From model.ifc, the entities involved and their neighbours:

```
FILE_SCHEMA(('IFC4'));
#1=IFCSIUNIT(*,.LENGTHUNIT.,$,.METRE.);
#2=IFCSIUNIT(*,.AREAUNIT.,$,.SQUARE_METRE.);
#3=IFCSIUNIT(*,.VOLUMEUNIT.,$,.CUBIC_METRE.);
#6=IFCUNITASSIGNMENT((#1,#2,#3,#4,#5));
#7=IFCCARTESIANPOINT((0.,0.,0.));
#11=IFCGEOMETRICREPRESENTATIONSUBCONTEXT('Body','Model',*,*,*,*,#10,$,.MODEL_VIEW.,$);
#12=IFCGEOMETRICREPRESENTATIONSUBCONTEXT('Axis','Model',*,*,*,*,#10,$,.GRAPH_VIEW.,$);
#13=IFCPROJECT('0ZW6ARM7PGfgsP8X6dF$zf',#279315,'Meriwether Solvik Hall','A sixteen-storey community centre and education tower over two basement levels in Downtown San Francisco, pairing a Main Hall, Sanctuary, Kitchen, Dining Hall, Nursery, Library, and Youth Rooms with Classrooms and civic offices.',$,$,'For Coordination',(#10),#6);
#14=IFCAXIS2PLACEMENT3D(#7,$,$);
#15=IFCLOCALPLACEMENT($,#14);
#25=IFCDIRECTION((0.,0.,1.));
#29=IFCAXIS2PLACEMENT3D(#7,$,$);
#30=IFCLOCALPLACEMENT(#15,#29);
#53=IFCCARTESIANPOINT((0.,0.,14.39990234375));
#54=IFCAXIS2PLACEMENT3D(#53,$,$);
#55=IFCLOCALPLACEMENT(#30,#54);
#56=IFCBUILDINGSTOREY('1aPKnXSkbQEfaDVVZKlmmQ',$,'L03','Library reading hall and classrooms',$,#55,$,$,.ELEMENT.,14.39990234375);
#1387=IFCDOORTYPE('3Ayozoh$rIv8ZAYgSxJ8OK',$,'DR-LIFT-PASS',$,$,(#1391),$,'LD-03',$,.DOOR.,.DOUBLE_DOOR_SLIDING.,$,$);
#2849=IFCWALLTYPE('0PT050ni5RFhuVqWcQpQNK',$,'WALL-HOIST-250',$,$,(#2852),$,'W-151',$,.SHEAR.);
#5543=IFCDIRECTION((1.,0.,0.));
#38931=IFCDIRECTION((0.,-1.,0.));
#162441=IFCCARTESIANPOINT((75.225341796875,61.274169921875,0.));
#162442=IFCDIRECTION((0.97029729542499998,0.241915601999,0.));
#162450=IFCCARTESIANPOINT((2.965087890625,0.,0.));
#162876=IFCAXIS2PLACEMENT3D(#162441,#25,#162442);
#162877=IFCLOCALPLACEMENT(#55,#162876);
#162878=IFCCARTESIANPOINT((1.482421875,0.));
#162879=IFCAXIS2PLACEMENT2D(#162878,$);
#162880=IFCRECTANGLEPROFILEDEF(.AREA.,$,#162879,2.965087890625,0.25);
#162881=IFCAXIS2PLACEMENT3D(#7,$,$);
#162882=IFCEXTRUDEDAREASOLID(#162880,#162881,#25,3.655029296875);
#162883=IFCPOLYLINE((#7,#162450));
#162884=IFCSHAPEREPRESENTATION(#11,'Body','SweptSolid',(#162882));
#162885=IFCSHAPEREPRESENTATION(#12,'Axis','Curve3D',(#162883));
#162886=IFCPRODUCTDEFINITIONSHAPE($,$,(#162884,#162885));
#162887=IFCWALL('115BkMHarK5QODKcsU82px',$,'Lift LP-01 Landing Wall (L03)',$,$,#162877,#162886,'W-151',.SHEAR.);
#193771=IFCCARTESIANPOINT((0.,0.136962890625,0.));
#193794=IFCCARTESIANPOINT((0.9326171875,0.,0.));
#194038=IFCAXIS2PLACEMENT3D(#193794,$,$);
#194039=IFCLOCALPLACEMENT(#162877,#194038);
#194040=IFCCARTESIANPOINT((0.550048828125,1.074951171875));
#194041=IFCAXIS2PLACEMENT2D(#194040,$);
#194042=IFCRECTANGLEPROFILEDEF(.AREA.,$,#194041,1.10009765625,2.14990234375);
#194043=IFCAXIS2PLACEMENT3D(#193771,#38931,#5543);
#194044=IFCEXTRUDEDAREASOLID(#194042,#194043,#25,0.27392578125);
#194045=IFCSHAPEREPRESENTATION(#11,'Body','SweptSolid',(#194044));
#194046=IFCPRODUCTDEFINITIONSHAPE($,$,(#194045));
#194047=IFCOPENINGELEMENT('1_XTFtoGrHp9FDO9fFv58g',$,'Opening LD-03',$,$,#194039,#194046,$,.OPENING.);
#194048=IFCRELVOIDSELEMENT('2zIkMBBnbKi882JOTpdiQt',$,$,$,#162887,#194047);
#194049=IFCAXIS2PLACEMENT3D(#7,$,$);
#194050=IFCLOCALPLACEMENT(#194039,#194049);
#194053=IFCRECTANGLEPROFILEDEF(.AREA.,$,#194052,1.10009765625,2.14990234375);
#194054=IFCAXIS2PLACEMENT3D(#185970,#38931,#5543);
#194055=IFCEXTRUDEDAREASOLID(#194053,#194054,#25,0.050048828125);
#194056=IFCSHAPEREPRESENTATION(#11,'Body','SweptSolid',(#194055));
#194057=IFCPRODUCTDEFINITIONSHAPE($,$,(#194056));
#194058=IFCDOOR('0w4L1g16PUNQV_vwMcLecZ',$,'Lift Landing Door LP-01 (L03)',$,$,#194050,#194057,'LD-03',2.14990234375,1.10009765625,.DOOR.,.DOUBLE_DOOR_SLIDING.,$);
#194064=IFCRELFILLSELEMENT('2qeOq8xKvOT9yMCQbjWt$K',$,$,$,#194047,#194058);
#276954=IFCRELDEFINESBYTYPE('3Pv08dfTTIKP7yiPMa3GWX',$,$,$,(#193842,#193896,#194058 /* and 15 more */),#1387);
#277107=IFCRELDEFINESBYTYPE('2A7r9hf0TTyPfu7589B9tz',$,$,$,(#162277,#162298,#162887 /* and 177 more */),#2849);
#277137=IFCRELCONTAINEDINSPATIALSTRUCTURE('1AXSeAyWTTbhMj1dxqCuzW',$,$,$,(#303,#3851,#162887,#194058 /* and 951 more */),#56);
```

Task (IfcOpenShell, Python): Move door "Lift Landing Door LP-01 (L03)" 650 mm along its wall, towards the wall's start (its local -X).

```python
import ifcopenshell
import ifcopenshell.api.geometry
import ifcopenshell.util.placement
import ifcopenshell.util.unit

model = ifcopenshell.open("model.ifc")
unit_scale = ifcopenshell.util.unit.calculate_unit_scale(model)

door = model.by_id(194058)
opening = door.FillsVoids[0].RelatingOpeningElement
wall = opening.VoidsElements[0].RelatingBuildingElement

wall_matrix = ifcopenshell.util.placement.get_local_placement(wall.ObjectPlacement)
shift = wall_matrix[:3, 0] * -0.65 / unit_scale
before = ifcopenshell.util.placement.get_local_placement(door.ObjectPlacement)[:3, 3].copy()

# The door is placed relative to its opening, so it follows when the opening moves.
matrix = ifcopenshell.util.placement.get_local_placement(opening.ObjectPlacement)
matrix[:3, 3] += shift
ifcopenshell.api.geometry.edit_object_placement(
    model, product=opening, matrix=matrix, is_si=False, should_transform_children=True
)

after = ifcopenshell.util.placement.get_local_placement(door.ObjectPlacement)[:3, 3]
print("door moved by", (after - before).round(3) + 0.0)

model.write("model_rev.ifc")
```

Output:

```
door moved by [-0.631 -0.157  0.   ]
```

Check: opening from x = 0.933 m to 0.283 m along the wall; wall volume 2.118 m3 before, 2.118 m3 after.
